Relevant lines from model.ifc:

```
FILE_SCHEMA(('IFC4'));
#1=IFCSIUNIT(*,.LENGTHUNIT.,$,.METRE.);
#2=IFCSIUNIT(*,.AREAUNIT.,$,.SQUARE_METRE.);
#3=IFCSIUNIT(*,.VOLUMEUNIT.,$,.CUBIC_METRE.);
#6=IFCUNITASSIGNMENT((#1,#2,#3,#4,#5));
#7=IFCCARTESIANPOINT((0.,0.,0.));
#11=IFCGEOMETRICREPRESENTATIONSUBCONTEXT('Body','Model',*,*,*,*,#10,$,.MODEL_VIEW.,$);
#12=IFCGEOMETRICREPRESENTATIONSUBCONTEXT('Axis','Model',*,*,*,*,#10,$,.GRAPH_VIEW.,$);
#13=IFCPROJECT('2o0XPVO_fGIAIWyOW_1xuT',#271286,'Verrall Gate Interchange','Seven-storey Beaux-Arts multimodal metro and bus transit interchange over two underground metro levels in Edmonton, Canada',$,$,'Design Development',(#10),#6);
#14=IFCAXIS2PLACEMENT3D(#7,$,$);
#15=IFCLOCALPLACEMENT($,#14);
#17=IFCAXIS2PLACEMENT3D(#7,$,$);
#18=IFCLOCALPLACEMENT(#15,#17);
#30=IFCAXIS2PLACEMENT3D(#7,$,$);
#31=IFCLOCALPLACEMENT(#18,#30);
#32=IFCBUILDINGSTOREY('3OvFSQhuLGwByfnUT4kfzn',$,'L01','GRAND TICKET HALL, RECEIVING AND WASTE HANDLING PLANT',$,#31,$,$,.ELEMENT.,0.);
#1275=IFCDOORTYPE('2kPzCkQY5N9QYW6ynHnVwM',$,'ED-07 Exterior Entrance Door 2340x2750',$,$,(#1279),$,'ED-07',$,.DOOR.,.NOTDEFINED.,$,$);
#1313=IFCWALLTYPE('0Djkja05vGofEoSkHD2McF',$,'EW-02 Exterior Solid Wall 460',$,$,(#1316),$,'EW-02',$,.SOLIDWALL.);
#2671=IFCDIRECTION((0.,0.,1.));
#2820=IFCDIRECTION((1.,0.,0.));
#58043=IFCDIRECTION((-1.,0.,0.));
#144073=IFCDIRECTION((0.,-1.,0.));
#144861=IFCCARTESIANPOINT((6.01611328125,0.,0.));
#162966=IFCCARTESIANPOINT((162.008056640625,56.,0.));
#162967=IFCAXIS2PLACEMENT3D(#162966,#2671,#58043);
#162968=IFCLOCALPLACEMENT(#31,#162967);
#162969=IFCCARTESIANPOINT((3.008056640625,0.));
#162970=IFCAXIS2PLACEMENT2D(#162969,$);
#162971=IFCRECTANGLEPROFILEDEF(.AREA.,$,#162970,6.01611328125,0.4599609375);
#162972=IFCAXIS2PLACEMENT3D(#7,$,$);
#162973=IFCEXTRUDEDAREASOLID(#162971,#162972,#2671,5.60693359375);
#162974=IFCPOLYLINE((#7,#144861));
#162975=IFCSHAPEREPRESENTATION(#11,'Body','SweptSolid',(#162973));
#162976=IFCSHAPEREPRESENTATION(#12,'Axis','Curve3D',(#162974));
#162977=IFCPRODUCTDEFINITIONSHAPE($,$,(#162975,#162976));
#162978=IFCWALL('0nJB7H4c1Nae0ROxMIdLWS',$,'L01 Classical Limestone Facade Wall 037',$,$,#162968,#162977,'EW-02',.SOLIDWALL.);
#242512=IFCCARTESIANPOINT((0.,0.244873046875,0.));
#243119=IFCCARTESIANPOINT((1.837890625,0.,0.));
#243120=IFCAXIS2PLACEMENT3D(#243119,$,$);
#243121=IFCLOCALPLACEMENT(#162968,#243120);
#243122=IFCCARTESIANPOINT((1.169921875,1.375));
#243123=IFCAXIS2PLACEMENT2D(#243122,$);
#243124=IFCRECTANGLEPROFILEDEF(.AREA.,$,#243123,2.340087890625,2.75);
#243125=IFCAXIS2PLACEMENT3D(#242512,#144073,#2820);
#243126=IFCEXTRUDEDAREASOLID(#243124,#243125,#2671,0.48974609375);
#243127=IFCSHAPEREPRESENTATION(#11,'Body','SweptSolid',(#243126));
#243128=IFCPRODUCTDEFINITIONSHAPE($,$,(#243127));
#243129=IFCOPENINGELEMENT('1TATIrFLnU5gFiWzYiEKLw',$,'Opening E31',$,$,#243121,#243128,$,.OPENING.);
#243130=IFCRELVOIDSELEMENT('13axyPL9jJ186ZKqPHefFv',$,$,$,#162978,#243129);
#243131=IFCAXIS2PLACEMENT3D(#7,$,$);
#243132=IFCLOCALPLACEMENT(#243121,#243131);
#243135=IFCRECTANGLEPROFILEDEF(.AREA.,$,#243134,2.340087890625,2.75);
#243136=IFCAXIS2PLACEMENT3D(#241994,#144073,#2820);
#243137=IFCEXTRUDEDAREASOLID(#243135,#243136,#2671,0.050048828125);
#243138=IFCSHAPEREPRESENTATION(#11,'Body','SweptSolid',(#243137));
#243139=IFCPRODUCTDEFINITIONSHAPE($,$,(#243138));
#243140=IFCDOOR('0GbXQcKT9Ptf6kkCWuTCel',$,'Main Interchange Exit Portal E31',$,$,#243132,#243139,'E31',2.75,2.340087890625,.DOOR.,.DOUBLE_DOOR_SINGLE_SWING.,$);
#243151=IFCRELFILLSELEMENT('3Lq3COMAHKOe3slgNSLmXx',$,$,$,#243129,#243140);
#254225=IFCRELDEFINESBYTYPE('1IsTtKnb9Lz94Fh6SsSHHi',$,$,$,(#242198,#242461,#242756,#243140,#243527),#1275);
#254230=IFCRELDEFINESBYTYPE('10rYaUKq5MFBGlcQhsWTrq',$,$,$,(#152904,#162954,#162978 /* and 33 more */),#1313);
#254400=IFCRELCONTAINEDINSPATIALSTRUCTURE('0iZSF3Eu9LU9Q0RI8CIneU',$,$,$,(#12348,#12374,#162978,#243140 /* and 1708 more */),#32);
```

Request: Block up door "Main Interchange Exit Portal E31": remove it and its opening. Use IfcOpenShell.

```python
import ifcopenshell
import ifcopenshell.api.feature
import ifcopenshell.api.root
import ifcopenshell.geom
import ifcopenshell.util.shape

model = ifcopenshell.open("model.ifc")
settings = ifcopenshell.geom.settings()


def volume(element):
    """Net volume in cubic metres, openings subtracted."""
    shape = ifcopenshell.geom.create_shape(settings, element)
    return ifcopenshell.util.shape.get_volume(shape.geometry)


door = model.by_guid("0GbXQcKT9Ptf6kkCWuTCel")
opening = door.FillsVoids[0].RelatingOpeningElement
wall = opening.VoidsElements[0].RelatingBuildingElement
before = volume(wall)

ifcopenshell.api.root.remove_product(model, product=door)
ifcopenshell.api.feature.remove_feature(model, feature=opening)

after = volume(wall)

print(f"wall volume {before:.3f} -> {after:.3f} m3")

model.write("model_rev.ifc")
```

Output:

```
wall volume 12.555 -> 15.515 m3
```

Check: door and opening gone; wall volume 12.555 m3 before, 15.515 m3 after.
